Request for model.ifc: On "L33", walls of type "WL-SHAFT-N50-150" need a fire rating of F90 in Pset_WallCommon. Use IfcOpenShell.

First a look at what the model holds.

```python
import ifcopenshell
import ifcopenshell.util.element

model = ifcopenshell.open("model.ifc")
print(model.schema)
storey = next(s for s in model.by_type("IfcBuildingStorey") if s.Name == "L33")
walls = [e for e in ifcopenshell.util.element.get_decomposition(storey) if e.is_a("IfcWall")]
seen = {}
for e in walls:
    element_type = ifcopenshell.util.element.get_type(e)
    key = (element_type.Name if element_type != e and element_type else None, ifcopenshell.util.element.get_pset(e, "Pset_WallCommon", "FireRating"))
    seen[key] = seen.get(key, 0) + 1
for (name, value), count in sorted(seen.items(), key=str):
    print(count, "x", name, "|", value)
```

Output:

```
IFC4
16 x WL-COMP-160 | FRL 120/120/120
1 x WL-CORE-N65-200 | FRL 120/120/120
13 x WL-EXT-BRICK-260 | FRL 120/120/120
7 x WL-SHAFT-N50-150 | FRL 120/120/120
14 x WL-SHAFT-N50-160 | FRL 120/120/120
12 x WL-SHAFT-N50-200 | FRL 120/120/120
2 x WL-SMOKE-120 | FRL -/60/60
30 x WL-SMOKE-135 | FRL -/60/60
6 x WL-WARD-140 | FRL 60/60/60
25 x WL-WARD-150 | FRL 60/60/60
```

```python
import ifcopenshell
import ifcopenshell.api.pset
import ifcopenshell.util.element

model = ifcopenshell.open("model.ifc")

storey = next(s for s in model.by_type("IfcBuildingStorey") if s.Name == "L33")
walls = [e for e in ifcopenshell.util.element.get_decomposition(storey) if e.is_a("IfcWall")]

count = 0
for e in walls:
    element_type = ifcopenshell.util.element.get_type(e)
    if element_type in (None, e) or element_type.Name != "WL-SHAFT-N50-150":
        continue
    # add_pset returns the element's existing set when there is one.
    pset = ifcopenshell.api.pset.add_pset(model, product=e, name="Pset_WallCommon")
    ifcopenshell.api.pset.edit_pset(model, pset=pset, properties={"FireRating": "F90"})
    count += 1

print(count, "walls updated")

model.write("model-out.ifc")
```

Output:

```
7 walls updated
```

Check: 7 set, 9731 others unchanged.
